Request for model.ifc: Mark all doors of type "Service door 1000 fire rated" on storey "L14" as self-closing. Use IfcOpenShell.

First a look at what the model holds.

```python
import ifcopenshell
import ifcopenshell.util.element

model = ifcopenshell.open("model.ifc")
print(model.schema)
storey = next(s for s in model.by_type("IfcBuildingStorey") if s.Name == "L14")
doors = [e for e in ifcopenshell.util.element.get_decomposition(storey) if e.is_a("IfcDoor")]
seen = {}
for e in doors:
    element_type = ifcopenshell.util.element.get_type(e)
    key = (element_type.Name if element_type != e and element_type else None, ifcopenshell.util.element.get_pset(e, "Pset_DoorCommon", "SelfClosing"))
    seen[key] = seen.get(key, 0) + 1
for (name, value), count in sorted(seen.items(), key=str):
    print(count, "x", name, "|", value)
```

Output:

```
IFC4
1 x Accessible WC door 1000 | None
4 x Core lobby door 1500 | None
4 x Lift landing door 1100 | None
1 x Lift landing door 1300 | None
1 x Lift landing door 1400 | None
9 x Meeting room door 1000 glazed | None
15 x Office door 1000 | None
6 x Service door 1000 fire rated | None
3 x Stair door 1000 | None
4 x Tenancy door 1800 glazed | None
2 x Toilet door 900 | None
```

```python
import ifcopenshell
import ifcopenshell.api.pset
import ifcopenshell.util.element

model = ifcopenshell.open("model.ifc")

storey = next(s for s in model.by_type("IfcBuildingStorey") if s.Name == "L14")
doors = [e for e in ifcopenshell.util.element.get_decomposition(storey) if e.is_a("IfcDoor")]

count = 0
for e in doors:
    element_type = ifcopenshell.util.element.get_type(e)
    if element_type in (None, e) or element_type.Name != "Service door 1000 fire rated":
        continue
    # add_pset returns the element's existing set when there is one.
    pset = ifcopenshell.api.pset.add_pset(model, product=e, name="Pset_DoorCommon")
    ifcopenshell.api.pset.edit_pset(model, pset=pset, properties={"SelfClosing": True})
    count += 1

print(count, "doors updated")

model.write("model_updated.ifc")
```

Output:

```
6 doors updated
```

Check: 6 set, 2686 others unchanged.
